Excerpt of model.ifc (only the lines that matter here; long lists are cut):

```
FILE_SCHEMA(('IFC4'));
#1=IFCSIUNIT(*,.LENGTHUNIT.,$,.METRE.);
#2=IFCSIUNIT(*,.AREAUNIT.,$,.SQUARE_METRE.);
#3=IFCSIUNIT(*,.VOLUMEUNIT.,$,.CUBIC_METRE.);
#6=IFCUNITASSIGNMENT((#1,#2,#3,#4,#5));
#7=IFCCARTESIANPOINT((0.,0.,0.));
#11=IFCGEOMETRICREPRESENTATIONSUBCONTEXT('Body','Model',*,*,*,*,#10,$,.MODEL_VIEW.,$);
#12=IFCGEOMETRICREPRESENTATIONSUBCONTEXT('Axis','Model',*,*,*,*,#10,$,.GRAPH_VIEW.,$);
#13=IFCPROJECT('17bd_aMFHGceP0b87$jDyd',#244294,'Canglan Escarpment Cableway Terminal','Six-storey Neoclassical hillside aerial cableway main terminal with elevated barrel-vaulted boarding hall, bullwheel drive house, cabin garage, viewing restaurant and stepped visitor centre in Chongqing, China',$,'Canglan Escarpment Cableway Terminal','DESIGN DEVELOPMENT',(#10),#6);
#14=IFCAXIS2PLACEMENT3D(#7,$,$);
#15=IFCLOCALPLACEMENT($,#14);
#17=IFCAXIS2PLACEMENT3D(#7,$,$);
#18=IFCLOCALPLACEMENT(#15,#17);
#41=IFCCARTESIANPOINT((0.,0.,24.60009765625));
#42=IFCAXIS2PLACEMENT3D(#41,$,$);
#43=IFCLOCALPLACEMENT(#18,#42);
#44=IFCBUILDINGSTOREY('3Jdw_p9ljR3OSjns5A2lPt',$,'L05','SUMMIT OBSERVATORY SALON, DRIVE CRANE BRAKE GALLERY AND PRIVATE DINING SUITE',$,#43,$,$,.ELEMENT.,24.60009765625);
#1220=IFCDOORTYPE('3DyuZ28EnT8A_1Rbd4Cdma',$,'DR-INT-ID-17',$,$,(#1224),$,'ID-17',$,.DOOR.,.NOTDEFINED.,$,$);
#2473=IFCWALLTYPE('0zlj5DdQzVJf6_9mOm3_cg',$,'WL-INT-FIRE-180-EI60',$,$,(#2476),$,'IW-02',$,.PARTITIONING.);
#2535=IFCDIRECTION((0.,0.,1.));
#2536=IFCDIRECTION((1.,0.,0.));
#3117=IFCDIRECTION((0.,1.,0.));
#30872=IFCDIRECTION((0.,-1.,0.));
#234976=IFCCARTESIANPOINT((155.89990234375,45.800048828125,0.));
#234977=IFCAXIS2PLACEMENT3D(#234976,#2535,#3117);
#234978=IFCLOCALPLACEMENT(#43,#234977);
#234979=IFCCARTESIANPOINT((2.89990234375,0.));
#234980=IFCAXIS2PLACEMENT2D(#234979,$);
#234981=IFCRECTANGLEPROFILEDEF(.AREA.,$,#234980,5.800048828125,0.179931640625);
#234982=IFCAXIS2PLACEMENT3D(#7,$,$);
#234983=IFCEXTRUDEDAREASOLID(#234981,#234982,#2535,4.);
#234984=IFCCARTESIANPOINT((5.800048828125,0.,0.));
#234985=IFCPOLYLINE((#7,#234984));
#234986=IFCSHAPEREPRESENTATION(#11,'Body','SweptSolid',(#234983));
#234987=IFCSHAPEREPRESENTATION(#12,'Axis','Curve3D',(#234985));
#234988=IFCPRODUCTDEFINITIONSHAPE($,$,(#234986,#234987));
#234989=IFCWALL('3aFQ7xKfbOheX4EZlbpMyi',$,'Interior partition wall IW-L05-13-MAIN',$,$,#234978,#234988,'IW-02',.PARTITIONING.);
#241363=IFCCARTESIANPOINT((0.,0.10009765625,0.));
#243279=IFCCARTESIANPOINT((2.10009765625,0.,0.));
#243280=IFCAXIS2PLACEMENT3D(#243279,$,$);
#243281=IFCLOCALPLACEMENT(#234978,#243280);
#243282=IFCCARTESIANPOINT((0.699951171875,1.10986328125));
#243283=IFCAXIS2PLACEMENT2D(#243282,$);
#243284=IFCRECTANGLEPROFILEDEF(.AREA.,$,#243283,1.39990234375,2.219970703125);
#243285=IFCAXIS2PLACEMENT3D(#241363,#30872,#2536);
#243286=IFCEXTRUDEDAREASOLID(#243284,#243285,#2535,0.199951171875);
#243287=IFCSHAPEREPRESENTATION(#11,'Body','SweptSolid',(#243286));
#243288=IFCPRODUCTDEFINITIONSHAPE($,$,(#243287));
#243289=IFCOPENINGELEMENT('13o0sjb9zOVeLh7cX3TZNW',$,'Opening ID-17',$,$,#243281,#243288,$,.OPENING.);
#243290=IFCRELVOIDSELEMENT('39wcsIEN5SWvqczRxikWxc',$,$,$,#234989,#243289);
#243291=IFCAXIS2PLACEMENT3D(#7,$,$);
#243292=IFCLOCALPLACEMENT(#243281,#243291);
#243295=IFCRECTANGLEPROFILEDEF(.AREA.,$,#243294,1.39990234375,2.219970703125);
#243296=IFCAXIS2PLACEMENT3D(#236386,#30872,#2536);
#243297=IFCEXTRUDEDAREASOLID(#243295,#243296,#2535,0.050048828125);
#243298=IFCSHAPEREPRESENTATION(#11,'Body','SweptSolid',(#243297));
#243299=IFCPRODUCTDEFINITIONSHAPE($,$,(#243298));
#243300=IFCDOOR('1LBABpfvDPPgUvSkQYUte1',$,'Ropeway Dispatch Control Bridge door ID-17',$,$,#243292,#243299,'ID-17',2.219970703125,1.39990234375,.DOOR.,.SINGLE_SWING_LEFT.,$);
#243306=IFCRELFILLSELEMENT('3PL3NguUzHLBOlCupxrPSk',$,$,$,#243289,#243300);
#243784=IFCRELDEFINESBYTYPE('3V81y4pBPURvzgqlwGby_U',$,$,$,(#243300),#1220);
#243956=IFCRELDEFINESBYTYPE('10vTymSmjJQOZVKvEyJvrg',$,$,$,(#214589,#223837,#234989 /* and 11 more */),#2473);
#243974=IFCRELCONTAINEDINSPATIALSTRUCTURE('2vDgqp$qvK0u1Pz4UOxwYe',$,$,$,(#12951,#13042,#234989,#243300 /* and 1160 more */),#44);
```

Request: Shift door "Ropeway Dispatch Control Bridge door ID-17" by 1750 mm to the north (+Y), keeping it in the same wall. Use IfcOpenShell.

```python
import ifcopenshell
import ifcopenshell.api.geometry
import ifcopenshell.util.placement

model = ifcopenshell.open("model.ifc")

door = model.by_guid("1LBABpfvDPPgUvSkQYUte1")
opening = door.FillsVoids[0].RelatingOpeningElement
wall = opening.VoidsElements[0].RelatingBuildingElement

wall_matrix = ifcopenshell.util.placement.get_local_placement(wall.ObjectPlacement)
shift = wall_matrix[:3, 0] * 1.75
before = ifcopenshell.util.placement.get_local_placement(door.ObjectPlacement)[:3, 3].copy()

# The door is placed relative to its opening, so it follows when the opening moves.
matrix = ifcopenshell.util.placement.get_local_placement(opening.ObjectPlacement)
matrix[:3, 3] += shift
ifcopenshell.api.geometry.edit_object_placement(
    model, product=opening, matrix=matrix, is_si=False, should_transform_children=True
)

after = ifcopenshell.util.placement.get_local_placement(door.ObjectPlacement)[:3, 3]
print("door moved by", (after - before).round(3) + 0.0)

model.write("model_v2.ifc")
```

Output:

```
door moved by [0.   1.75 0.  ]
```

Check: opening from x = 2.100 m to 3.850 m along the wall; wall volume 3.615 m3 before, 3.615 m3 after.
